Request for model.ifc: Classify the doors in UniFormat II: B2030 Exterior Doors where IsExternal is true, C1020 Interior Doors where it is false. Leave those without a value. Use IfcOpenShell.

First a look at what the model holds.

```python
import ifcopenshell
import ifcopenshell.util.element

model = ifcopenshell.open("model.ifc")
print(model.schema)
print("classifications:", [c.Name for c in model.by_type("IfcClassification")])
values = [ifcopenshell.util.element.get_pset(e, "Pset_DoorCommon", "IsExternal") for e in model.by_type("IfcDoor")]
for value in (True, False, None):
    print("IsExternal", value, values.count(value))
```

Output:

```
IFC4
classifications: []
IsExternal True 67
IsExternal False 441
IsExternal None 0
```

```python
import ifcopenshell
import ifcopenshell.api.classification
import ifcopenshell.util.element

model = ifcopenshell.open("model.ifc")

system = ifcopenshell.api.classification.add_classification(model, classification="UniFormat II")

doors = model.by_type("IfcDoor")
external = {e: ifcopenshell.util.element.get_pset(e, "Pset_DoorCommon", "IsExternal") for e in doors}
for flag, code, name in ((True, "B2030", "Exterior Doors"), (False, "C1020", "Interior Doors")):
    products = [e for e in doors if external[e] is flag]
    ifcopenshell.api.classification.add_reference(
        model, products=products, classification=system, identification=code, name=name
    )
    print(code, len(products))

model.write("model_v2.ifc")
```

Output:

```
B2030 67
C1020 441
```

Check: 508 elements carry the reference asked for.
